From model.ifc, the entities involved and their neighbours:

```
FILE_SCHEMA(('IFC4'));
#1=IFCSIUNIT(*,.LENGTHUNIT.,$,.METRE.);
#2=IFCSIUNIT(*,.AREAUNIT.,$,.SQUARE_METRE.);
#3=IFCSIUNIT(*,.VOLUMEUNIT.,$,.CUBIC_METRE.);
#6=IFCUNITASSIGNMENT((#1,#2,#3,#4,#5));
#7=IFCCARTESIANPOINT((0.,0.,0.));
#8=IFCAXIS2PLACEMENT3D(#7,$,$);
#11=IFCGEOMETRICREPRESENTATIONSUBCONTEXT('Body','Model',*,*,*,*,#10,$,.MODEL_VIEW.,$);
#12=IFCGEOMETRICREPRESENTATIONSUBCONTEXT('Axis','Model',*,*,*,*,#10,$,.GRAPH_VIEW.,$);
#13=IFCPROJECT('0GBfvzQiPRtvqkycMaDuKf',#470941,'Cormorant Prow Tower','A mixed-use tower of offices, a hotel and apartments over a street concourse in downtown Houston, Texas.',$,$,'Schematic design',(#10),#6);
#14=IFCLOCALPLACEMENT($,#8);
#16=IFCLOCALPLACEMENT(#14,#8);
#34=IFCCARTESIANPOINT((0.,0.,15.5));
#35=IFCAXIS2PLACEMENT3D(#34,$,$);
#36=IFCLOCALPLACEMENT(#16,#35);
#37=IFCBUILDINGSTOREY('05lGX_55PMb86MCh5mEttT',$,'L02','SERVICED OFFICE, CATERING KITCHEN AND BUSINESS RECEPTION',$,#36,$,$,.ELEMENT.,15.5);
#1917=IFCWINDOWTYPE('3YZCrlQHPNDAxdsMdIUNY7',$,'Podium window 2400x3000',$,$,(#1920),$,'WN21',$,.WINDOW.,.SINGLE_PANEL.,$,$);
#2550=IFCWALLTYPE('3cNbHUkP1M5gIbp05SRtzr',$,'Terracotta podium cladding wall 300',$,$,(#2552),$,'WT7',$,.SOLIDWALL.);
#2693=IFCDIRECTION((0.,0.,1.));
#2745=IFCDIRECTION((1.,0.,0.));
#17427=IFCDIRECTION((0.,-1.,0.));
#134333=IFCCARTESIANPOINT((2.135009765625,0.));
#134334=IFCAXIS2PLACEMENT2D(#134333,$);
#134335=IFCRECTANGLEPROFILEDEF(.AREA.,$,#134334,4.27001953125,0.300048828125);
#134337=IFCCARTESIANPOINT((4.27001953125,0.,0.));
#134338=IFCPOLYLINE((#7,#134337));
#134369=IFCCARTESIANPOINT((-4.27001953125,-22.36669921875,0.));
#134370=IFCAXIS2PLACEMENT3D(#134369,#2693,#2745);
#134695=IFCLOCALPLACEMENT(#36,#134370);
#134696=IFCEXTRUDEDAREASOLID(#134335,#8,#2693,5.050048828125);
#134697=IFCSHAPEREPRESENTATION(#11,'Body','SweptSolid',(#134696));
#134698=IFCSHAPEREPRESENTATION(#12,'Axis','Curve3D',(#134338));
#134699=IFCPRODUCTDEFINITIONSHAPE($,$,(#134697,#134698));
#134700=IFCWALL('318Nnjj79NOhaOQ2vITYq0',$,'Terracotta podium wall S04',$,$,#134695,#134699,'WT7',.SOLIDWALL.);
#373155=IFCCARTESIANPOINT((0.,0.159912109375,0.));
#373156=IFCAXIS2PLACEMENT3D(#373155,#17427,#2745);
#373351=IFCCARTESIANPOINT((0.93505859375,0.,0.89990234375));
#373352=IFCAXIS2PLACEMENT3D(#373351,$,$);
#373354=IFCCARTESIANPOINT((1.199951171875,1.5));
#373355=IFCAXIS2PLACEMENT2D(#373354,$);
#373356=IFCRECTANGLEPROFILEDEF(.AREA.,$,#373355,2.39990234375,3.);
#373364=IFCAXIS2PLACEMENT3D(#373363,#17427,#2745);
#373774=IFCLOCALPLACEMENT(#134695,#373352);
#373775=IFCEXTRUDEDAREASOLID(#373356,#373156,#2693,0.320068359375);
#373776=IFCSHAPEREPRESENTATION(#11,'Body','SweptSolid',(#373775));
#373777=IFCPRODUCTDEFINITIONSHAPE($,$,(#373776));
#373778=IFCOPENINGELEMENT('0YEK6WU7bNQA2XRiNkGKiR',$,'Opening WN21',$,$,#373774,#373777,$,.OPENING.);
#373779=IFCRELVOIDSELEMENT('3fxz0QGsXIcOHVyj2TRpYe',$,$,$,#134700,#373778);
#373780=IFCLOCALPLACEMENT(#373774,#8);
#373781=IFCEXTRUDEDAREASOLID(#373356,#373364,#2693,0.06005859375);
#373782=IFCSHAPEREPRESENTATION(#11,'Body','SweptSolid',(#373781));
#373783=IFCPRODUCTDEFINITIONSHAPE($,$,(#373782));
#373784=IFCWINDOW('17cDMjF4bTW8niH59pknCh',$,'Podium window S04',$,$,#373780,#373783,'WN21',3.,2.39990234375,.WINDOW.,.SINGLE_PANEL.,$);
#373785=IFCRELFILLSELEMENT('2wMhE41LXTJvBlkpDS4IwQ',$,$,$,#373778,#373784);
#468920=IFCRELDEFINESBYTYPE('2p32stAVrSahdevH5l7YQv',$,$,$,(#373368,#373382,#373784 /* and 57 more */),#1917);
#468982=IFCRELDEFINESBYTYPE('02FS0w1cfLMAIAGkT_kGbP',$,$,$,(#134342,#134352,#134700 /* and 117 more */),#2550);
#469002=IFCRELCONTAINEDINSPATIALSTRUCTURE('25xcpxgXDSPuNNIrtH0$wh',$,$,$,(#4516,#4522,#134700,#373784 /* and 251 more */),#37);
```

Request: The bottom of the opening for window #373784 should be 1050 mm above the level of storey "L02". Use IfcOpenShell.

```python
import numpy as np
import ifcopenshell
import ifcopenshell.api.geometry
import ifcopenshell.geom
import ifcopenshell.util.element
import ifcopenshell.util.placement
import ifcopenshell.util.shape
import ifcopenshell.util.unit

model = ifcopenshell.open("model.ifc")
unit_scale = ifcopenshell.util.unit.calculate_unit_scale(model)

window = model.by_guid("17cDMjF4bTW8niH59pknCh")
opening = window.FillsVoids[0].RelatingOpeningElement
storey = ifcopenshell.util.element.get_container(window, ifc_class="IfcBuildingStorey")
level = ifcopenshell.util.placement.get_local_placement(storey.ObjectPlacement)[2, 3]

# The opening's origin need not be at the sill, so measure its lowest point.
shape = ifcopenshell.geom.create_shape(ifcopenshell.geom.settings(), opening)
bottom = ifcopenshell.util.shape.get_shape_bottom_elevation(shape, shape.geometry) / unit_scale
dz = level + 1.05 / unit_scale - bottom

shift = np.array([0.0, 0.0, dz])
# The window is placed relative to its opening, so it follows when the opening moves.
matrix = ifcopenshell.util.placement.get_local_placement(opening.ObjectPlacement)
matrix[:3, 3] += shift
ifcopenshell.api.geometry.edit_object_placement(
    model, product=opening, matrix=matrix, is_si=False, should_transform_children=True
)

print(f"moved by {dz * unit_scale:+.3f} m")

model.write("model-out.ifc")
```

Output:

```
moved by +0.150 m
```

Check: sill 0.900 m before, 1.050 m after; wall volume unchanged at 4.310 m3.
